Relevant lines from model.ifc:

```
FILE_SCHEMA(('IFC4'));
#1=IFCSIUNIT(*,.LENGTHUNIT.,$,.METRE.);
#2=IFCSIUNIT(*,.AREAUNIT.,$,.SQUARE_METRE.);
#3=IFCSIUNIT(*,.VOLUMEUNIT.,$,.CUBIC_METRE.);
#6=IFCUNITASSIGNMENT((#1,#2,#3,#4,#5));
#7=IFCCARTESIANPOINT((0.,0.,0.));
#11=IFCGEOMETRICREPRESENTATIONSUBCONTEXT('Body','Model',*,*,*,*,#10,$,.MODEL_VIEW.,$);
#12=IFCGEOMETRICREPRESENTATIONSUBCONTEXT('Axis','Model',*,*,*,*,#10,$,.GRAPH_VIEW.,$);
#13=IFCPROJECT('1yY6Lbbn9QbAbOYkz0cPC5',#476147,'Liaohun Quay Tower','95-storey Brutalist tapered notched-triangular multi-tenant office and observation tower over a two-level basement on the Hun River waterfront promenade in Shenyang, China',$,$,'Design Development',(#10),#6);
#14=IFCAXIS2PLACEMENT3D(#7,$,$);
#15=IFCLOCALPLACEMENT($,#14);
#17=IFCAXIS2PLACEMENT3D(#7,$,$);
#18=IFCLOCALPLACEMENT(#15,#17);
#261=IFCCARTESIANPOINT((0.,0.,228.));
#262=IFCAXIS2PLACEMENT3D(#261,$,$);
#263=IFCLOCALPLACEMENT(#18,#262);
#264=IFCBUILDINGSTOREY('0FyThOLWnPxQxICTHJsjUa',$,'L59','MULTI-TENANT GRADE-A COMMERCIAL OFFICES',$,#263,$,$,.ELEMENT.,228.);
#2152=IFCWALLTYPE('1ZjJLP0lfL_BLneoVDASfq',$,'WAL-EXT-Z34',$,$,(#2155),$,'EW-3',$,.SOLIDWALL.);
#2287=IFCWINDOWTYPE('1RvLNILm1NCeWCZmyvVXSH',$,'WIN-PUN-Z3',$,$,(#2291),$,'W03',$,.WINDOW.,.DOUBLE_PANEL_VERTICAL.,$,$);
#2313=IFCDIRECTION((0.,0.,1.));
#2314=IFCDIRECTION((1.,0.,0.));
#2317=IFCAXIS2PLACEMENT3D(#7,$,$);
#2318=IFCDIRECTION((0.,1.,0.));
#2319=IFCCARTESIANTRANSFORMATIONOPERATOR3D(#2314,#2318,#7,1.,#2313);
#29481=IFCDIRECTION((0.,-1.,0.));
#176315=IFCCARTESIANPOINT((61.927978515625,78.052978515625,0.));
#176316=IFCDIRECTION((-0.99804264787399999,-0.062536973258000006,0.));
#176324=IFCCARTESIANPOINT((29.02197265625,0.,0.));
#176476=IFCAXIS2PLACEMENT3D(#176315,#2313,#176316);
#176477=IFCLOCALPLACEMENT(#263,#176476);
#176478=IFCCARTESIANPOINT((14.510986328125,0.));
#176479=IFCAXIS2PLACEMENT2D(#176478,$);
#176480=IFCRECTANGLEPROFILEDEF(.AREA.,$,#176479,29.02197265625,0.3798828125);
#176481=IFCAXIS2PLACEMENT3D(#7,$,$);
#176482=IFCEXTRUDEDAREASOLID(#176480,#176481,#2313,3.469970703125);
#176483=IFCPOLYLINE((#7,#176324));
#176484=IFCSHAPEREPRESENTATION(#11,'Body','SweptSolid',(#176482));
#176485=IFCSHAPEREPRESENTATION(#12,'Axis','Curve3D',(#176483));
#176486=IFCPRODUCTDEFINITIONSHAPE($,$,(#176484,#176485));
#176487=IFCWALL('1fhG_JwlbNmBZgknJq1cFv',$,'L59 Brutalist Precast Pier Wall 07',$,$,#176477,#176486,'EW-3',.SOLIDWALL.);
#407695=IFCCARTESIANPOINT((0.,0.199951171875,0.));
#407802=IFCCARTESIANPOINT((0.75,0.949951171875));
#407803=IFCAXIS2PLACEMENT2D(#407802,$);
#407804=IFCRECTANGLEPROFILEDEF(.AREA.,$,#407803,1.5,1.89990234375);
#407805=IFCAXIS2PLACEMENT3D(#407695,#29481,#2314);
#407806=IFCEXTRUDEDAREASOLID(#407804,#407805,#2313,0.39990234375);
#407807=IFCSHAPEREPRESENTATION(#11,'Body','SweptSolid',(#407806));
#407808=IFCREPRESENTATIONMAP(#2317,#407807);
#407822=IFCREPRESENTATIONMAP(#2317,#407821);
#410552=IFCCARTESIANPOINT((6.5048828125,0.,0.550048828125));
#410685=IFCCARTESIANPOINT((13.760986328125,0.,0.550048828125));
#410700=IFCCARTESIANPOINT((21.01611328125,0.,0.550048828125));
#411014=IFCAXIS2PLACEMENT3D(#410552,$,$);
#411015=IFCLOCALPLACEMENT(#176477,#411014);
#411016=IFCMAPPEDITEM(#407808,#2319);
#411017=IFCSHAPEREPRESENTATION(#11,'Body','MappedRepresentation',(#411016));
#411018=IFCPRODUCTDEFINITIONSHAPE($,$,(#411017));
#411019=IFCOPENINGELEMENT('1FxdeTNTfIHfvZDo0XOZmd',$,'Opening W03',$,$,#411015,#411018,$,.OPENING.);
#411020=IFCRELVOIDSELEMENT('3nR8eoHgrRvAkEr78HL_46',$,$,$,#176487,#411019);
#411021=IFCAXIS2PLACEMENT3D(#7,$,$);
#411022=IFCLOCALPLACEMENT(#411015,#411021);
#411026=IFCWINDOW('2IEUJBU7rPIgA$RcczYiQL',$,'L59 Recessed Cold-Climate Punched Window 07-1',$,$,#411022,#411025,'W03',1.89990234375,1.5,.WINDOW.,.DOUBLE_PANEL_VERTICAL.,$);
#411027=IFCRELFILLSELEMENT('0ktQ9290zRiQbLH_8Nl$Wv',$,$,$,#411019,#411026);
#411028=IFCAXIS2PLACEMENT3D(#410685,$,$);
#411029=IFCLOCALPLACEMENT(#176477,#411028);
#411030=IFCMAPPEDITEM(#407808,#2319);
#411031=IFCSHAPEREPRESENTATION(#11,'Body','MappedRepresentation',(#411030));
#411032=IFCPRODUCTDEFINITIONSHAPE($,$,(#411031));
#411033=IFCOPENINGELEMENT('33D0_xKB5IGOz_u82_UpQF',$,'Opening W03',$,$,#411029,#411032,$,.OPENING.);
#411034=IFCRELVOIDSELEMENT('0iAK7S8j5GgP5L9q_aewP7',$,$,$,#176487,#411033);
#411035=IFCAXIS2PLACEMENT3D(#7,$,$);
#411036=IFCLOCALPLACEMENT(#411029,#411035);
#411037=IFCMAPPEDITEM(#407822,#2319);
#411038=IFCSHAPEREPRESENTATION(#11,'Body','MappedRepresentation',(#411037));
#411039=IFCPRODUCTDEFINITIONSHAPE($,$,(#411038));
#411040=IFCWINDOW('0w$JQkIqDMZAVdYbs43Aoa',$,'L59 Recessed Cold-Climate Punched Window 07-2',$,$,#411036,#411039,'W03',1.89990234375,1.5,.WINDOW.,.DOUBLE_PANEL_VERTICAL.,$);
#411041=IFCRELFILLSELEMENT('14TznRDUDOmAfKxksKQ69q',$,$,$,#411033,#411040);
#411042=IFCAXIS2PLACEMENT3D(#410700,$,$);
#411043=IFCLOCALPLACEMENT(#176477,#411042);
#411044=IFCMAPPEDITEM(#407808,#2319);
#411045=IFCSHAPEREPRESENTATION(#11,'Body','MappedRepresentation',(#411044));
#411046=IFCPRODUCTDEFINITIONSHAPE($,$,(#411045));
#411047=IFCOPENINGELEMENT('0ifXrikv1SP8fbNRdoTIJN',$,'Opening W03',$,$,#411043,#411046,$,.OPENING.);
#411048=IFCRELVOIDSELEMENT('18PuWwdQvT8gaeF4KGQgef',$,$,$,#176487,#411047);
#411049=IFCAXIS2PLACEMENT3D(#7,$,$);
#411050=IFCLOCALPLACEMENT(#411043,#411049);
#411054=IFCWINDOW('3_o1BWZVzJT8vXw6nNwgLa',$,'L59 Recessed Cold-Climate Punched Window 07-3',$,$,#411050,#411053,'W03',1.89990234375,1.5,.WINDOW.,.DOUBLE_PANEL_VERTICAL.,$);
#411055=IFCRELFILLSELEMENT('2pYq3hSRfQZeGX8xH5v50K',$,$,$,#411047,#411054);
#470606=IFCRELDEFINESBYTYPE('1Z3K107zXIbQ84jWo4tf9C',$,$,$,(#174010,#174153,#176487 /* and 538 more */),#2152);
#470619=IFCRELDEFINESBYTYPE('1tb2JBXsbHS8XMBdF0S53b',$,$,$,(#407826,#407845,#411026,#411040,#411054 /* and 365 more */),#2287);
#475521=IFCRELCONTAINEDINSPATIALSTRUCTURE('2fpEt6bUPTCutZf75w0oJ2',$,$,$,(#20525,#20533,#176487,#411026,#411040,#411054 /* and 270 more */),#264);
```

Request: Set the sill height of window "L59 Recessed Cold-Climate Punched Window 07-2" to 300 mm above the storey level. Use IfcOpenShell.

```python
import numpy as np
import ifcopenshell
import ifcopenshell.api.geometry
import ifcopenshell.geom
import ifcopenshell.util.element
import ifcopenshell.util.placement
import ifcopenshell.util.shape
import ifcopenshell.util.unit

model = ifcopenshell.open("model.ifc")
unit_scale = ifcopenshell.util.unit.calculate_unit_scale(model)

window = model.by_guid("0w$JQkIqDMZAVdYbs43Aoa")
opening = window.FillsVoids[0].RelatingOpeningElement
storey = ifcopenshell.util.element.get_container(window, ifc_class="IfcBuildingStorey")
level = ifcopenshell.util.placement.get_local_placement(storey.ObjectPlacement)[2, 3]

# The opening's origin need not be at the sill, so measure its lowest point.
shape = ifcopenshell.geom.create_shape(ifcopenshell.geom.settings(), opening)
bottom = ifcopenshell.util.shape.get_shape_bottom_elevation(shape, shape.geometry) / unit_scale
dz = level + 0.3 - bottom

shift = np.array([0.0, 0.0, dz])
# The window is placed relative to its opening, so it follows when the opening moves.
matrix = ifcopenshell.util.placement.get_local_placement(opening.ObjectPlacement)
matrix[:3, 3] += shift
ifcopenshell.api.geometry.edit_object_placement(
    model, product=opening, matrix=matrix, is_si=False, should_transform_children=True
)

print(f"moved by {dz * unit_scale:+.3f} m")

model.write("model_edited.ifc")
```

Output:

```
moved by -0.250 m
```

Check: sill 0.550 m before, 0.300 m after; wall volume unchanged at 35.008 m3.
